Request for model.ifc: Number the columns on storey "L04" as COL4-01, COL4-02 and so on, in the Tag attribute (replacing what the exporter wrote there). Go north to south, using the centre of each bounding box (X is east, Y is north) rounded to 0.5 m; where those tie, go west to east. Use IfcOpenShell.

First a look at what the model holds.

```python
import ifcopenshell
import ifcopenshell.util.element
import ifcopenshell.util.placement

model = ifcopenshell.open("model.ifc")
print(model.schema)
storey = next(s for s in model.by_type("IfcBuildingStorey") if s.Name == "L04")
columns = [e for e in ifcopenshell.util.element.get_decomposition(storey) if e.is_a("IfcColumn")]
for e in sorted(columns, key=lambda e: e.id()):
    origin = ifcopenshell.util.placement.get_local_placement(e.ObjectPlacement)[:3, 3]
    print(e.id(), e.Tag, e.Name, origin.round(2) + 0.0, sep=" | ")
```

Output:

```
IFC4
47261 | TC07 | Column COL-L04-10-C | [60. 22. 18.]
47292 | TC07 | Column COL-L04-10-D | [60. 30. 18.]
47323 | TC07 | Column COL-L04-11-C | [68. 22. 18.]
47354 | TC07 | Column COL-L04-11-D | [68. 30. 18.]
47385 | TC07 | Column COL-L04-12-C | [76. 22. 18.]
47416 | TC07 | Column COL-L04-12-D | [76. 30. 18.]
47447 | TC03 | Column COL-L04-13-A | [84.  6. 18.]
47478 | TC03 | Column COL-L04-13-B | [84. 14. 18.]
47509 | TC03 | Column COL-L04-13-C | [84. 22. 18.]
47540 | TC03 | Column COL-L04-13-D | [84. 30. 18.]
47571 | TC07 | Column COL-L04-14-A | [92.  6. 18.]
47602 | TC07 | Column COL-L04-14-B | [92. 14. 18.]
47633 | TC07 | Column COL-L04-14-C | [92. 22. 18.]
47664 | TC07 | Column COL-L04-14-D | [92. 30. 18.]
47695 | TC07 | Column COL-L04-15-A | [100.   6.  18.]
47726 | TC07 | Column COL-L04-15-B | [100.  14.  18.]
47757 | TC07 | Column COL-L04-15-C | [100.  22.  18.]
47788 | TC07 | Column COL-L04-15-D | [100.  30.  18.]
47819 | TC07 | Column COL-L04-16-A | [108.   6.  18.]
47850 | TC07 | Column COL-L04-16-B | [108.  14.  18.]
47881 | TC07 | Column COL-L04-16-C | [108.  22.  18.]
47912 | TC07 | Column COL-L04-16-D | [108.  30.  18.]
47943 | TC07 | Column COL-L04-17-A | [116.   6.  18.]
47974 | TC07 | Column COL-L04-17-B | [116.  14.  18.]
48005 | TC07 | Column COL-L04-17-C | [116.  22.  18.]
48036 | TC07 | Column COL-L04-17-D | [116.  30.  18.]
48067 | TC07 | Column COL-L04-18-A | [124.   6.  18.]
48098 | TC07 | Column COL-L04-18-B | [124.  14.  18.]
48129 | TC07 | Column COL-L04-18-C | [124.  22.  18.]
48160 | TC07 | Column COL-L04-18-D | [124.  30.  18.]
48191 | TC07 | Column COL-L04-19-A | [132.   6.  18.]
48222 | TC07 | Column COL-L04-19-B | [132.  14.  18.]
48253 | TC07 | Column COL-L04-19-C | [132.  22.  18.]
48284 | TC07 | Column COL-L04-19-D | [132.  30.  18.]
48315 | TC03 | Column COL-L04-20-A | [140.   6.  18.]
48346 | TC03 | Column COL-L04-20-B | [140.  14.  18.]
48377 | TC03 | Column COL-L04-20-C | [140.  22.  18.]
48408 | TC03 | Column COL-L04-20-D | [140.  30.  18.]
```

```python
import ifcopenshell
import ifcopenshell.geom
import ifcopenshell.util.element
import ifcopenshell.util.shape

model = ifcopenshell.open("model.ifc")
settings = ifcopenshell.geom.settings()
settings.set("use-world-coords", True)


def centre(element):
    shape = ifcopenshell.geom.create_shape(settings, element)
    return ifcopenshell.util.shape.get_bbox_centroid(shape.geometry)


storey = next(s for s in model.by_type("IfcBuildingStorey") if s.Name == "L04")
columns = [e for e in ifcopenshell.util.element.get_decomposition(storey) if e.is_a("IfcColumn")]

# Insertion points can sit at a corner or the storey origin, so sort by the geometry (in metres).
centres = {e: centre(e) for e in columns}
columns.sort(key=lambda e: (-round(centres[e][1] / 0.5), centres[e][0]))

for i, e in enumerate(columns, start=1):
    number = f"COL4-{i:02d}"
    e.Tag = number
    print(e.id(), number)

model.write("model_edited.ifc")
```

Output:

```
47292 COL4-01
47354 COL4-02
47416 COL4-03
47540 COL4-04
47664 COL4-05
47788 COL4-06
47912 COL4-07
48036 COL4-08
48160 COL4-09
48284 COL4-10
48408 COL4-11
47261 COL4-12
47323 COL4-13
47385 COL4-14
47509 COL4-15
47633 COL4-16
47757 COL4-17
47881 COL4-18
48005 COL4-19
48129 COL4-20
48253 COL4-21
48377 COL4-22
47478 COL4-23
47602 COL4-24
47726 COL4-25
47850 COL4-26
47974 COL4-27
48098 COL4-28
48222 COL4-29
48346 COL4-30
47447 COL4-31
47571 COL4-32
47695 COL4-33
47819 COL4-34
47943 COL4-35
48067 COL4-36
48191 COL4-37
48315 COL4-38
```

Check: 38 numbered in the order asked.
